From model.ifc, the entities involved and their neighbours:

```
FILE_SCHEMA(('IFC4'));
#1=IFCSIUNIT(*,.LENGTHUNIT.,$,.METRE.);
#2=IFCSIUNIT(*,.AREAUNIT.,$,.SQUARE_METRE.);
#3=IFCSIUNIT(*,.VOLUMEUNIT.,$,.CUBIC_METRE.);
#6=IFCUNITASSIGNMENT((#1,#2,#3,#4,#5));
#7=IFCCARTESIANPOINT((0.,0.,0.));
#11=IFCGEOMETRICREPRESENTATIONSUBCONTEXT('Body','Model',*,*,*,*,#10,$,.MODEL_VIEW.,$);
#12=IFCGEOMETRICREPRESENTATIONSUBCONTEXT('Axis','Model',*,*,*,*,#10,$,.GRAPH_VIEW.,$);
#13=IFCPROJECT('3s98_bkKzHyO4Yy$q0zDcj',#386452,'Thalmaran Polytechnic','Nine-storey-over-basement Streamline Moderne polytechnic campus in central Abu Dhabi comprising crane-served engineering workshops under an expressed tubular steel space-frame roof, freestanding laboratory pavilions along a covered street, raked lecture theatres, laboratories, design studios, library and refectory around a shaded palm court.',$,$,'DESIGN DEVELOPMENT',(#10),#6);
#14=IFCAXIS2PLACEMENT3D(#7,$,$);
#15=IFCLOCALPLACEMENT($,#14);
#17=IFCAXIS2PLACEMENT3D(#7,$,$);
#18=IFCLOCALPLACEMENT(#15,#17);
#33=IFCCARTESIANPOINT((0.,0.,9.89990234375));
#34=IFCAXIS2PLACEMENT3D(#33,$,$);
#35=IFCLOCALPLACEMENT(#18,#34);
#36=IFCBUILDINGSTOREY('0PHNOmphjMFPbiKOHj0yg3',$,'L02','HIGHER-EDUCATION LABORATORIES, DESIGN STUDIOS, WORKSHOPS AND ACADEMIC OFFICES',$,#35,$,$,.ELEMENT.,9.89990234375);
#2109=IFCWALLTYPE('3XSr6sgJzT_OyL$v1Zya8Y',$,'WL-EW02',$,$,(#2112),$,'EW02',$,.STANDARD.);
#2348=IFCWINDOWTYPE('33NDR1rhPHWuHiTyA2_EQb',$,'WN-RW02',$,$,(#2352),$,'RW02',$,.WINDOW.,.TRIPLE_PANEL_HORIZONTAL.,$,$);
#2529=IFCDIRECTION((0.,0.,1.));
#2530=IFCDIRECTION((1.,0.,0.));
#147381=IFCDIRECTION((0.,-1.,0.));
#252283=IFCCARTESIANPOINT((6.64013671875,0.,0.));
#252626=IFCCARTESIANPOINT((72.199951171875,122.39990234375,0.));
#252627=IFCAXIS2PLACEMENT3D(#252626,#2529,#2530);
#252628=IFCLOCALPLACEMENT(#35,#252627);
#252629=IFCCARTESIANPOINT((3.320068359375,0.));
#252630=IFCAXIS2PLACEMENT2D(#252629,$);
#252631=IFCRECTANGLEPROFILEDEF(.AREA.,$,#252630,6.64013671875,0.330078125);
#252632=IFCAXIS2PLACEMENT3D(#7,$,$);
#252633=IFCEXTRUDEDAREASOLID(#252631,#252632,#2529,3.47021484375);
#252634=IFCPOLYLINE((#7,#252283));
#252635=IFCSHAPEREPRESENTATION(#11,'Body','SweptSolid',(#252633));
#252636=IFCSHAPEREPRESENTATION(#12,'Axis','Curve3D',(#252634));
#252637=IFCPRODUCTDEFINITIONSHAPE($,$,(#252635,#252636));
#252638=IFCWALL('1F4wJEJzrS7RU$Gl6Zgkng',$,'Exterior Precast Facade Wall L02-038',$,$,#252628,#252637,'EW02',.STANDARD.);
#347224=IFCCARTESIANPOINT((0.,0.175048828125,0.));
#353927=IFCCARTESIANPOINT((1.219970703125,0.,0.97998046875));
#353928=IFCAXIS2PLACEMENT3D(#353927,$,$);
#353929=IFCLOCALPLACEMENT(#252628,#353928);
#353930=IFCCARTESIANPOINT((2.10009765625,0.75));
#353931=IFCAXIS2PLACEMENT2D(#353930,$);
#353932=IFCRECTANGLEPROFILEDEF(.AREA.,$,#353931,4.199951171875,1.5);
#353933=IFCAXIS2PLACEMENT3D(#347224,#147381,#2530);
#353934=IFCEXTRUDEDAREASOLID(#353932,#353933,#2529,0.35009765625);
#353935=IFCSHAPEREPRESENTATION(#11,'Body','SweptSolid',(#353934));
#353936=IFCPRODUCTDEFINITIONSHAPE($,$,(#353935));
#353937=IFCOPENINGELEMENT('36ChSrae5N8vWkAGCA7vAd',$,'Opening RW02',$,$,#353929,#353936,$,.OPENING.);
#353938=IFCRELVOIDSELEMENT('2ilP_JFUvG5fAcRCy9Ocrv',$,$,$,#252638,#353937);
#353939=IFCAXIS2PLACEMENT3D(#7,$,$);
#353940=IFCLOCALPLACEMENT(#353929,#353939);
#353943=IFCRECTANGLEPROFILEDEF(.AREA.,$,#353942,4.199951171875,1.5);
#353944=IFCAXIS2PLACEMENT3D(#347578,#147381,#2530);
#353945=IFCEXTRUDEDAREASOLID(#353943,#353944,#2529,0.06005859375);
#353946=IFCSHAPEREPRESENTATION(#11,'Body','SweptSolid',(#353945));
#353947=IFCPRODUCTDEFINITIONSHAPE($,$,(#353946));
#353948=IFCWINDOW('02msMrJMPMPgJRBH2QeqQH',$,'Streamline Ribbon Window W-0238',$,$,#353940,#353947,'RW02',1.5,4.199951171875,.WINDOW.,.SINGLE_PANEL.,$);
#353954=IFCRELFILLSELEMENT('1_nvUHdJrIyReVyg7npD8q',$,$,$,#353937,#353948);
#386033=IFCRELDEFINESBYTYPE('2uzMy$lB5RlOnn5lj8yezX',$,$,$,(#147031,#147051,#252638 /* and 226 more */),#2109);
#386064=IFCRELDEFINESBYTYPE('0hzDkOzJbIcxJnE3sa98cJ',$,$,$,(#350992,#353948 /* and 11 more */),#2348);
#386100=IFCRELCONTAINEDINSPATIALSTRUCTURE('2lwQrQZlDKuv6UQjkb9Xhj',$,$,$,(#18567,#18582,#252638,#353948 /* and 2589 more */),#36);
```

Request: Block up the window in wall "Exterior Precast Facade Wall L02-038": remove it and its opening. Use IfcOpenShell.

```python
import ifcopenshell
import ifcopenshell.api.feature
import ifcopenshell.api.root
import ifcopenshell.geom
import ifcopenshell.util.shape

model = ifcopenshell.open("model.ifc")
settings = ifcopenshell.geom.settings()


def volume(element):
    """Net volume in cubic metres, openings subtracted."""
    shape = ifcopenshell.geom.create_shape(settings, element)
    return ifcopenshell.util.shape.get_volume(shape.geometry)


window = model.by_id(353948)
opening = window.FillsVoids[0].RelatingOpeningElement
wall = opening.VoidsElements[0].RelatingBuildingElement
before = volume(wall)

ifcopenshell.api.root.remove_product(model, product=window)
ifcopenshell.api.feature.remove_feature(model, feature=opening)

after = volume(wall)

print(f"wall volume {before:.3f} -> {after:.3f} m3")

model.write("model_updated.ifc")
```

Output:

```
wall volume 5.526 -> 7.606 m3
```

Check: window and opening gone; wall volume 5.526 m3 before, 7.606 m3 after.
